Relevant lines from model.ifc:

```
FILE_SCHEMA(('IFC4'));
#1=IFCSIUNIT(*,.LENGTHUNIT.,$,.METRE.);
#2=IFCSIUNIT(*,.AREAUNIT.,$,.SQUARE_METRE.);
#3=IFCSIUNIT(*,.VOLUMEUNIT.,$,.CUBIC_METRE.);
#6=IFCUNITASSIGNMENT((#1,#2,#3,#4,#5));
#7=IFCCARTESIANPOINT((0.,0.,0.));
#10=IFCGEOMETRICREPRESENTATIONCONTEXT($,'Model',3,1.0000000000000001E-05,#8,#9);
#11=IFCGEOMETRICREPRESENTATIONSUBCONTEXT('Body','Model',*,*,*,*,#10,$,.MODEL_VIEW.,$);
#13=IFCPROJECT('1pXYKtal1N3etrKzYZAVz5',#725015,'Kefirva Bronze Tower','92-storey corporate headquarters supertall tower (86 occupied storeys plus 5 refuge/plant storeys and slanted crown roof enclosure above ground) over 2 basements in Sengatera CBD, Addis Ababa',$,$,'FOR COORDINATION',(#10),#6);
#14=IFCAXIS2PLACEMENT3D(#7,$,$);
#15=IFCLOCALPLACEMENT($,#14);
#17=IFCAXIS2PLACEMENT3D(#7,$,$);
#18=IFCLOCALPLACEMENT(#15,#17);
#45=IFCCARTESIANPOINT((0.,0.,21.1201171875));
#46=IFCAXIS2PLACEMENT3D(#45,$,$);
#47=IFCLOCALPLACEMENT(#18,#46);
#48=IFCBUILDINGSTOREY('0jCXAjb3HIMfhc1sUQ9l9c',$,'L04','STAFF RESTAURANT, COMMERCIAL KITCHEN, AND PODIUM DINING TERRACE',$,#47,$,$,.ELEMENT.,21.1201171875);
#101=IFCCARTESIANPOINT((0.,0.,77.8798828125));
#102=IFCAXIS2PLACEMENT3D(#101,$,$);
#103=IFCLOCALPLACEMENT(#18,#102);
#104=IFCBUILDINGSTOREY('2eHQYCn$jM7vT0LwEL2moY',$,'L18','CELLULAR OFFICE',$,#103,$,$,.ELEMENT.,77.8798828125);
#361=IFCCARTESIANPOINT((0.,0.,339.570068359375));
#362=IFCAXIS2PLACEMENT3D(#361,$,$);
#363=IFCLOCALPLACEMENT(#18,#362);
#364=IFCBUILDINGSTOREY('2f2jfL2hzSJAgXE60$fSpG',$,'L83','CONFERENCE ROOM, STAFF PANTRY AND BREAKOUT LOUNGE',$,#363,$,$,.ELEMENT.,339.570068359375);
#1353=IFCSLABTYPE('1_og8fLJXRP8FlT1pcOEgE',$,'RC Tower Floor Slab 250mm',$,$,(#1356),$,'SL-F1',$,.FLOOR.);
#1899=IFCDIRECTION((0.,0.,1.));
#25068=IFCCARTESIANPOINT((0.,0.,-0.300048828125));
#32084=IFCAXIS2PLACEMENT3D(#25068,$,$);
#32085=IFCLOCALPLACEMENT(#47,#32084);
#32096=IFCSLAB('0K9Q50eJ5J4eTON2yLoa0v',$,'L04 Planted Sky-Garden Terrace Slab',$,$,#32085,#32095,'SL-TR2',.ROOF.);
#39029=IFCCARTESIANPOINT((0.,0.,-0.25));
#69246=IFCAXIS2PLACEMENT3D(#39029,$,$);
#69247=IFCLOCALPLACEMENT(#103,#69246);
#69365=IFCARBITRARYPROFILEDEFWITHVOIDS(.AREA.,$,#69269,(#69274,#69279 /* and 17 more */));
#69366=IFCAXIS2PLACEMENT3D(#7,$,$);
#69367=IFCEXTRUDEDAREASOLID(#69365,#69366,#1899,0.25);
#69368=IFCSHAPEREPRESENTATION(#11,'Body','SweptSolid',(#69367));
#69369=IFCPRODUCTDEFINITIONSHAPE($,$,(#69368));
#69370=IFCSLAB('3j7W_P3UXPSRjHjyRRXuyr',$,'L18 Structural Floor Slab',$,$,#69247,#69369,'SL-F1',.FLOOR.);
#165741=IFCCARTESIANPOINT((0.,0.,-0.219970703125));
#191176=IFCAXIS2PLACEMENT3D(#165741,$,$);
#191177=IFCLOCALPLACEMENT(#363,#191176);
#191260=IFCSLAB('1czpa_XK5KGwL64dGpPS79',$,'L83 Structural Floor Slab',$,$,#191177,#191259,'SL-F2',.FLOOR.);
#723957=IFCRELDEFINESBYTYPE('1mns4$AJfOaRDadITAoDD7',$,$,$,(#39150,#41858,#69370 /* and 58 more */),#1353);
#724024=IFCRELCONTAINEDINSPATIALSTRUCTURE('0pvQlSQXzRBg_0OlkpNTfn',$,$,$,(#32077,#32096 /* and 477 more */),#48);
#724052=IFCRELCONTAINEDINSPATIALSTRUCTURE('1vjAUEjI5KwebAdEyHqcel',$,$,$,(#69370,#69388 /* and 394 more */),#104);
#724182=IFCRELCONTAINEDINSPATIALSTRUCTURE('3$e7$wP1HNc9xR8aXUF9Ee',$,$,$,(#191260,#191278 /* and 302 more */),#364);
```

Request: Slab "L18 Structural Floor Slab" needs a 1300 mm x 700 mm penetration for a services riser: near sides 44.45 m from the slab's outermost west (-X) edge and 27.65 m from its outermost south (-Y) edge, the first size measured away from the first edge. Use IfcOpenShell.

```python
import numpy as np
import ifcopenshell
import ifcopenshell.api.feature
import ifcopenshell.api.geometry
import ifcopenshell.api.root
import ifcopenshell.geom
import ifcopenshell.util.placement
import ifcopenshell.util.representation
import ifcopenshell.util.shape
import ifcopenshell.util.unit

model = ifcopenshell.open("model.ifc")
unit_scale = ifcopenshell.util.unit.calculate_unit_scale(model)
settings = ifcopenshell.geom.settings()


def volume(element):
    """Net volume in cubic metres, openings subtracted."""
    shape = ifcopenshell.geom.create_shape(settings, element)
    return ifcopenshell.util.shape.get_volume(shape.geometry)


slab = model.by_guid("3j7W_P3UXPSRjHjyRRXuyr")
before = volume(slab)

# Extent in the slab's own axes, in metres. The edges named are its -X and -Y sides.
slab_shape = ifcopenshell.geom.create_shape(settings, slab)
vertices = ifcopenshell.util.shape.get_vertices(slab_shape.geometry)
x_min, y_min, bottom = vertices.min(axis=0)
top = vertices[:, 2].max()

opening = ifcopenshell.api.root.create_entity(model, ifc_class="IfcOpeningElement", name="Services riser opening", predefined_type="OPENING")
context = ifcopenshell.util.representation.get_context(model, "Model", "Body", "MODEL_VIEW")
width, depth = 1.3, 0.7
outline = [(0.0, 0.0), (width, 0.0), (width, depth), (0.0, depth), (0.0, 0.0)]
# Overshoot both faces by 50 mm so the cut is clean.
shape = ifcopenshell.api.geometry.add_slab_representation(
    model, context=context, depth=top - bottom + 0.1, polyline=outline
)
ifcopenshell.api.geometry.assign_representation(model, product=opening, representation=shape)

matrix = ifcopenshell.util.placement.get_local_placement(slab.ObjectPlacement)
matrix[:, 3] = matrix @ np.append(np.array([x_min + 44.45, y_min + 27.65, bottom - 0.05]) / unit_scale, 1.0)
ifcopenshell.api.geometry.edit_object_placement(model, product=opening, matrix=matrix, is_si=False)
ifcopenshell.api.feature.add_feature(model, feature=opening, element=slab)

after = volume(slab)

print(f"slab volume {before:.3f} -> {after:.3f} m3")

model.write("model_updated.ifc")
```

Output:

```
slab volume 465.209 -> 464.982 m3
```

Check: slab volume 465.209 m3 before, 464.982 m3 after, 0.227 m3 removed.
